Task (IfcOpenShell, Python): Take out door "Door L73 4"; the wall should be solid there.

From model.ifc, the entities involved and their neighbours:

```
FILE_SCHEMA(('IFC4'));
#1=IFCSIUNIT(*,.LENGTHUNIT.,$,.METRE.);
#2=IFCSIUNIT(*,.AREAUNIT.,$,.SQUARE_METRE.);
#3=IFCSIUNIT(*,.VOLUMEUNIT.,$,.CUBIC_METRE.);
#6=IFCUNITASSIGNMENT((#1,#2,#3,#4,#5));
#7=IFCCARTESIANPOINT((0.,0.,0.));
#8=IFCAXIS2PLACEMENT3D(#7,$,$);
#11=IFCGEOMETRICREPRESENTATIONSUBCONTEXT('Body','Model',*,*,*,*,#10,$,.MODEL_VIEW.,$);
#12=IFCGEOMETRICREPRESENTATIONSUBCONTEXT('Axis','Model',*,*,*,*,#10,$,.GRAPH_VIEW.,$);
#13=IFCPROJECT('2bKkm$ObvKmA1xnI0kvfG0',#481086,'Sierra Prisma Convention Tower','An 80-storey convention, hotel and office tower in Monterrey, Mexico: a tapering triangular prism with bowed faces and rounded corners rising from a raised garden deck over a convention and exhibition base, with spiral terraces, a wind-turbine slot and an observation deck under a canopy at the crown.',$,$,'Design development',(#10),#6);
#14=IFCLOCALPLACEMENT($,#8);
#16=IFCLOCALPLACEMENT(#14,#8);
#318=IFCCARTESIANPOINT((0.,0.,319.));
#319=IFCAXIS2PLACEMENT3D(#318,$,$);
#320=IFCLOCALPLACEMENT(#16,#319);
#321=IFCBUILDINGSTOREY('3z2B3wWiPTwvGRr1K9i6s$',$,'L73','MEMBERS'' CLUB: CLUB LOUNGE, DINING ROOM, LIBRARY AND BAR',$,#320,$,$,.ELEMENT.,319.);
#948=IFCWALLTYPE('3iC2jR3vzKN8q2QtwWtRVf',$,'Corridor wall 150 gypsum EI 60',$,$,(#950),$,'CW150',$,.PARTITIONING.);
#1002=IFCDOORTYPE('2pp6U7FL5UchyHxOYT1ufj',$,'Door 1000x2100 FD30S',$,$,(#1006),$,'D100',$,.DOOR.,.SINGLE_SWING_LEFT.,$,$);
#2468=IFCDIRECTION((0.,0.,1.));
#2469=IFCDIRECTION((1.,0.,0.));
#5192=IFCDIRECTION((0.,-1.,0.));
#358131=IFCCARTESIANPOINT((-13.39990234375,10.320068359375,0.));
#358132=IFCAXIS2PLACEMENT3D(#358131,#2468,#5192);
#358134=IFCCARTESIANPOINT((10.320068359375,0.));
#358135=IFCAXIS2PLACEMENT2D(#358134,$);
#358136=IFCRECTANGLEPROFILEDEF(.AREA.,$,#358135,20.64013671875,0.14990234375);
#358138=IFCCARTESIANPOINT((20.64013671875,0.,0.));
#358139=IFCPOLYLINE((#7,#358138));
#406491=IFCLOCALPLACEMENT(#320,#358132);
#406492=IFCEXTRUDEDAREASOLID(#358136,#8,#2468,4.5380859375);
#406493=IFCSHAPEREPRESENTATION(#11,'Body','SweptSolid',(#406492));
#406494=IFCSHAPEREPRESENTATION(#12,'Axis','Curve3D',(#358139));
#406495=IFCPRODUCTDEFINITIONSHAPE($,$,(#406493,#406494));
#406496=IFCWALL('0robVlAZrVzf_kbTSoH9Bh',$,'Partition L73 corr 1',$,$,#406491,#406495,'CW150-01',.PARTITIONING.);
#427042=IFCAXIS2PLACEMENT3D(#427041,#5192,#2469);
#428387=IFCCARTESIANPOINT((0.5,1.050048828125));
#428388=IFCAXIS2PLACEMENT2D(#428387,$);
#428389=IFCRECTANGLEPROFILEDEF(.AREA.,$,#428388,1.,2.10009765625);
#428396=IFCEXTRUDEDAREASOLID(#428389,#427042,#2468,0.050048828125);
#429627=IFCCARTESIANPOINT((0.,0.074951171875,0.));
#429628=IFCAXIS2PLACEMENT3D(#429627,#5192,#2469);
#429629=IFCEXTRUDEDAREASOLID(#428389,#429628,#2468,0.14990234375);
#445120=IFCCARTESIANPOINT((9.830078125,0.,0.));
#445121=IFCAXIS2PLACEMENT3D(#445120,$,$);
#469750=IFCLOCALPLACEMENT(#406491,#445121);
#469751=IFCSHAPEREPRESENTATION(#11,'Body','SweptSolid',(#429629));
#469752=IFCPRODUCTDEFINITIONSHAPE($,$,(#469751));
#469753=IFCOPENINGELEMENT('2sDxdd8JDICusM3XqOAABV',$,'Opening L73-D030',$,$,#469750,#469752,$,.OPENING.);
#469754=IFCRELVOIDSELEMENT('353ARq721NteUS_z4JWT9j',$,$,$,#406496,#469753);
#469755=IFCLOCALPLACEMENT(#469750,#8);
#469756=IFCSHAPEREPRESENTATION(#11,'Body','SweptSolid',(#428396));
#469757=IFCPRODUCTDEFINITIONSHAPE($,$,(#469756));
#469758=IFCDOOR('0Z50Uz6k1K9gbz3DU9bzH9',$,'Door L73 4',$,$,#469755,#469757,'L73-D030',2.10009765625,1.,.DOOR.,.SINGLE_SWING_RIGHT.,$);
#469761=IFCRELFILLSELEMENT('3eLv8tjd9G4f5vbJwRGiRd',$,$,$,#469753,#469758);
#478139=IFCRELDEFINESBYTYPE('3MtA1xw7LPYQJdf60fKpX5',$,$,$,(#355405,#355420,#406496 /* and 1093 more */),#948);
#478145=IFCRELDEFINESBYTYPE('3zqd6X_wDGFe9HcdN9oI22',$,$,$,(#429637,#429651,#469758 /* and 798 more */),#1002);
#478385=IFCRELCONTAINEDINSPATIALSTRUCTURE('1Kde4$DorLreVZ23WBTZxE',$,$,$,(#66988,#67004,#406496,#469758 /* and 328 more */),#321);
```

```python
import ifcopenshell
import ifcopenshell.api.feature
import ifcopenshell.api.root
import ifcopenshell.geom
import ifcopenshell.util.shape

model = ifcopenshell.open("model.ifc")
settings = ifcopenshell.geom.settings()


def volume(element):
    """Net volume in cubic metres, openings subtracted."""
    shape = ifcopenshell.geom.create_shape(settings, element)
    return ifcopenshell.util.shape.get_volume(shape.geometry)


door = model.by_guid("0Z50Uz6k1K9gbz3DU9bzH9")
opening = door.FillsVoids[0].RelatingOpeningElement
wall = opening.VoidsElements[0].RelatingBuildingElement
before = volume(wall)

ifcopenshell.api.root.remove_product(model, product=door)
ifcopenshell.api.feature.remove_feature(model, feature=opening)

after = volume(wall)

print(f"wall volume {before:.3f} -> {after:.3f} m3")

model.write("model-out.ifc")
```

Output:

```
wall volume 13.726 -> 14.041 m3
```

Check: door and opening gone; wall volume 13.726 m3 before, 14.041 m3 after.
